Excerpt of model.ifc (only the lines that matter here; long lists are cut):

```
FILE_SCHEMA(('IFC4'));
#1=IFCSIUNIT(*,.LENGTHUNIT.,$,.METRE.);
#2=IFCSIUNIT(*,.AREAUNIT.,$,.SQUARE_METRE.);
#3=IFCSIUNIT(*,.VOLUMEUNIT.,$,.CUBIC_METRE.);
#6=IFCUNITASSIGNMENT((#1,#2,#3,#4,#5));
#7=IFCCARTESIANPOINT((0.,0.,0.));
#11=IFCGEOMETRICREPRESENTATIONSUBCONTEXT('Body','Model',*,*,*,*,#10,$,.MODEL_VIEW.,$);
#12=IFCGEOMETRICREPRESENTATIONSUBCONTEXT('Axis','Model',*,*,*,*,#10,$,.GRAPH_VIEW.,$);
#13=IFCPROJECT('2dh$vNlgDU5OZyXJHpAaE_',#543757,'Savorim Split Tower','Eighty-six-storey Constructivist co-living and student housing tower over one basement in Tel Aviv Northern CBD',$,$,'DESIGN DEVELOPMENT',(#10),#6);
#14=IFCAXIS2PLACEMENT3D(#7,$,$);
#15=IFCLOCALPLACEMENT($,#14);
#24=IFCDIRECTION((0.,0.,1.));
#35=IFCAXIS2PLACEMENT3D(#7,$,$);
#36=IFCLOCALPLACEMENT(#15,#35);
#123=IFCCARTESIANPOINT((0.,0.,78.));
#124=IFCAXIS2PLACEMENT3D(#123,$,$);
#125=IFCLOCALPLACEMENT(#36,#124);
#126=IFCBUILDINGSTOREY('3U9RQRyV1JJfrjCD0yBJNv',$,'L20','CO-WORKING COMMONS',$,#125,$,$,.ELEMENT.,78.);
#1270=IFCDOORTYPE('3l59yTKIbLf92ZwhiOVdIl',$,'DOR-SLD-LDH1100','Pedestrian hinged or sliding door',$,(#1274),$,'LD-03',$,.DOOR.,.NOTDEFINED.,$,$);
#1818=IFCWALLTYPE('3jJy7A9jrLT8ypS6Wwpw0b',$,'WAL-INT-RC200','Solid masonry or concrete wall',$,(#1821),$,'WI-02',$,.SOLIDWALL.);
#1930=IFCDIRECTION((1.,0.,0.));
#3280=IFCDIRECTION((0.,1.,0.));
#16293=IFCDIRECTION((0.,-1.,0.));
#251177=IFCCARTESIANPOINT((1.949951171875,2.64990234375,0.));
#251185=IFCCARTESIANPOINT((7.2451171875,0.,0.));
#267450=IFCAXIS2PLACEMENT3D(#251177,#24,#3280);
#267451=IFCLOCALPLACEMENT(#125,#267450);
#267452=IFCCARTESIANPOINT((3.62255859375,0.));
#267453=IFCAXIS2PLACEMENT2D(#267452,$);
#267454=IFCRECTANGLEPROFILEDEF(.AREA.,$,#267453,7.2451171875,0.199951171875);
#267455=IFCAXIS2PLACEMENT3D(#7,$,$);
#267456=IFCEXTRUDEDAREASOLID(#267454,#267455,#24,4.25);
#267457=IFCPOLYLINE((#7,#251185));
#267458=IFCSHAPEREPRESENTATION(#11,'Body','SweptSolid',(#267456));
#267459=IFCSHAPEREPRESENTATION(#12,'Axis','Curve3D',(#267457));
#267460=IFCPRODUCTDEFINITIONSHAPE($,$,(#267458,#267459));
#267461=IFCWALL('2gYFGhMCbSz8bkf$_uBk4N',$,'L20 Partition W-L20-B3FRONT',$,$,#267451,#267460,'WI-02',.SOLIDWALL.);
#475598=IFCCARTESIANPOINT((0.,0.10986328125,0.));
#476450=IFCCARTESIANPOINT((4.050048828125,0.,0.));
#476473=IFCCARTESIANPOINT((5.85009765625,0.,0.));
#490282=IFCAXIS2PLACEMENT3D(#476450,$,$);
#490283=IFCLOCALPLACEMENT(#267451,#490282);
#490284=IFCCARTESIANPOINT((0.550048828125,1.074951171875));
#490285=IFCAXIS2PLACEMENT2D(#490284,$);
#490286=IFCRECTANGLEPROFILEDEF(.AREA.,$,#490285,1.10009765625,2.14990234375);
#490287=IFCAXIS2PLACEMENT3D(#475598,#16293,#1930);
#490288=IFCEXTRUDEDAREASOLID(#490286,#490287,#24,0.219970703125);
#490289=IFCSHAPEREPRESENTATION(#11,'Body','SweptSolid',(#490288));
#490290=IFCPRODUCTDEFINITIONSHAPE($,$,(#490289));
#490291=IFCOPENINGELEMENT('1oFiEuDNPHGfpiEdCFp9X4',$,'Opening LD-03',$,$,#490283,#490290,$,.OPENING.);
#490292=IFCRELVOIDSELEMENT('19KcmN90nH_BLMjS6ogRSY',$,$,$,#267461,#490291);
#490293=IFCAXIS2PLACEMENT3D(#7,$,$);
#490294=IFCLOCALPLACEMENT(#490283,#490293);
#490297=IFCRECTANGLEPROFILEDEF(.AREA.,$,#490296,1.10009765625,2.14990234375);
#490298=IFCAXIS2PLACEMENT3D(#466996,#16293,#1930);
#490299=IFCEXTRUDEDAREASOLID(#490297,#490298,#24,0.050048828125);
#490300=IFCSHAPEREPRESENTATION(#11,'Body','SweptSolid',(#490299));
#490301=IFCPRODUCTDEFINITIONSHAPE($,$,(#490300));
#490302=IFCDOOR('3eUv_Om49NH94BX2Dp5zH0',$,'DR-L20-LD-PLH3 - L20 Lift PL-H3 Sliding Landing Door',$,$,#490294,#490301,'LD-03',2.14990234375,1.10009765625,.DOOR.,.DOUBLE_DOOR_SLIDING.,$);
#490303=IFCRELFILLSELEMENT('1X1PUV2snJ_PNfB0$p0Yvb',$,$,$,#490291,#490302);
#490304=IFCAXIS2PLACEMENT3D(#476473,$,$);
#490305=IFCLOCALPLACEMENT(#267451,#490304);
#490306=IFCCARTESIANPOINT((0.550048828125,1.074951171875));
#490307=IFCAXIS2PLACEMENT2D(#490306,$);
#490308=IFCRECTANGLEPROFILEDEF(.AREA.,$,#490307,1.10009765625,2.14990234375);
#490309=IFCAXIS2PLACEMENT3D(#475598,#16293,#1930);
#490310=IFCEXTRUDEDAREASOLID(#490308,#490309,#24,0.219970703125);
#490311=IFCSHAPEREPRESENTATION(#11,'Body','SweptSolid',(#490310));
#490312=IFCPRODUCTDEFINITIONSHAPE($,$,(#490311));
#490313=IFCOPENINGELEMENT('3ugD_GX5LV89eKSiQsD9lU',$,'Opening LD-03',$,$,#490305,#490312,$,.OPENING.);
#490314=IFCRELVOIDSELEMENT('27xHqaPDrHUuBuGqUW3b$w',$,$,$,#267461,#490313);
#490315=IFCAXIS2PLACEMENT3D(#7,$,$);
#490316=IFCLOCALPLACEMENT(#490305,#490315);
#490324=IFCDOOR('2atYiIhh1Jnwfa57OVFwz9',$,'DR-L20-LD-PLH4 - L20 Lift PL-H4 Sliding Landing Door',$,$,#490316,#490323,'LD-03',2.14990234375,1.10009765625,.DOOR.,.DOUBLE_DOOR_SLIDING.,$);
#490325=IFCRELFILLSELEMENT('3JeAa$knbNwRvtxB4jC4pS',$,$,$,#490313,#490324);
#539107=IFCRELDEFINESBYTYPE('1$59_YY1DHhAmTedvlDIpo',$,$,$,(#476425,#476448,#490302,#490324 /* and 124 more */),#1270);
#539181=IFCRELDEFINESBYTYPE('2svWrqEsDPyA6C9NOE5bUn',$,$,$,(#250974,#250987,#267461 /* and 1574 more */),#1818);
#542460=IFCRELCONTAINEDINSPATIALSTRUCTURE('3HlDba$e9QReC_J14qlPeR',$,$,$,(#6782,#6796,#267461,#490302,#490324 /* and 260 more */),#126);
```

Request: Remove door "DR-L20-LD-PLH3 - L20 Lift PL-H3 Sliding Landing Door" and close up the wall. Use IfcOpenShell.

```python
import ifcopenshell
import ifcopenshell.api.feature
import ifcopenshell.api.root
import ifcopenshell.geom
import ifcopenshell.util.shape

model = ifcopenshell.open("model.ifc")
settings = ifcopenshell.geom.settings()


def volume(element):
    """Net volume in cubic metres, openings subtracted."""
    shape = ifcopenshell.geom.create_shape(settings, element)
    return ifcopenshell.util.shape.get_volume(shape.geometry)


door = model.by_guid("3eUv_Om49NH94BX2Dp5zH0")
opening = door.FillsVoids[0].RelatingOpeningElement
wall = opening.VoidsElements[0].RelatingBuildingElement
before = volume(wall)

ifcopenshell.api.root.remove_product(model, product=door)
ifcopenshell.api.feature.remove_feature(model, feature=opening)

after = volume(wall)

print(f"wall volume {before:.3f} -> {after:.3f} m3")

model.write("model_rev.ifc")
```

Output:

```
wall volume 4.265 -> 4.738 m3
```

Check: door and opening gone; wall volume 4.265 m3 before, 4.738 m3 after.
